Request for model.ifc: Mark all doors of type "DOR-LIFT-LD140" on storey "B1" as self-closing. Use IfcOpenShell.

First a look at what the model holds.

```python
import ifcopenshell
import ifcopenshell.util.element

model = ifcopenshell.open("model.ifc")
print(model.schema)
storey = next(s for s in model.by_type("IfcBuildingStorey") if s.Name == "B1")
doors = [e for e in ifcopenshell.util.element.get_decomposition(storey) if e.is_a("IfcDoor")]
seen = {}
for e in doors:
    element_type = ifcopenshell.util.element.get_type(e)
    key = (element_type.Name if element_type != e and element_type else None, ifcopenshell.util.element.get_pset(e, "Pset_DoorCommon", "SelfClosing"))
    seen[key] = seen.get(key, 0) + 1
for (name, value), count in sorted(seen.items(), key=str):
    print(count, "x", name, "|", value)
```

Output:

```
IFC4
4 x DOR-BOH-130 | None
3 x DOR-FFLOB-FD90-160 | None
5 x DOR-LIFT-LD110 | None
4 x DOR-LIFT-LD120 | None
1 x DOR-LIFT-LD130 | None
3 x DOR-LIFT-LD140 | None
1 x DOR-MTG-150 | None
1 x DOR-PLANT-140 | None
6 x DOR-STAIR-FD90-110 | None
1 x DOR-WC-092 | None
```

```python
import ifcopenshell
import ifcopenshell.api.pset
import ifcopenshell.util.element

model = ifcopenshell.open("model.ifc")

storey = next(s for s in model.by_type("IfcBuildingStorey") if s.Name == "B1")
doors = [e for e in ifcopenshell.util.element.get_decomposition(storey) if e.is_a("IfcDoor")]

count = 0
for e in doors:
    element_type = ifcopenshell.util.element.get_type(e)
    if element_type in (None, e) or element_type.Name != "DOR-LIFT-LD140":
        continue
    # add_pset returns the element's existing set when there is one.
    pset = ifcopenshell.api.pset.add_pset(model, product=e, name="Pset_DoorCommon")
    ifcopenshell.api.pset.edit_pset(model, pset=pset, properties={"SelfClosing": True})
    count += 1

print(count, "doors updated")

model.write("model_edited.ifc")
```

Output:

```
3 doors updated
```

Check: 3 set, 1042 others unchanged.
